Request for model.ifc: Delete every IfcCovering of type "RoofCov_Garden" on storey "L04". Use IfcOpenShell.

First a look at what the model holds.

```python
import ifcopenshell
import ifcopenshell.util.element

model = ifcopenshell.open("model.ifc")
print(model.schema)
storey = next(s for s in model.by_type("IfcBuildingStorey") if s.Name == "L04")
coverings = [e for e in ifcopenshell.util.element.get_decomposition(storey) if e.is_a("IfcCovering")]
seen = {}
for e in coverings:
    element_type = ifcopenshell.util.element.get_type(e)
    name = element_type.Name if element_type not in (None, e) else None
    seen[name] = seen.get(name, 0) + 1
for name, count in sorted(seen.items(), key=str):
    print(count, "x", name)
```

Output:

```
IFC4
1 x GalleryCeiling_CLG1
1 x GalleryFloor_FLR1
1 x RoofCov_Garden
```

```python
import ifcopenshell
import ifcopenshell.api.root
import ifcopenshell.util.element

model = ifcopenshell.open("model.ifc")

storey = next(s for s in model.by_type("IfcBuildingStorey") if s.Name == "L04")
coverings = [e for e in ifcopenshell.util.element.get_decomposition(storey) if e.is_a("IfcCovering")]
targets = [e for e in coverings if (t := ifcopenshell.util.element.get_type(e)) not in (None, e) and t.Name == "RoofCov_Garden"]

for e in targets:
    ifcopenshell.api.root.remove_product(model, product=e)
print(len(targets), "removed")

model.write("model_v2.ifc")
```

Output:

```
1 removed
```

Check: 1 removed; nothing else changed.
